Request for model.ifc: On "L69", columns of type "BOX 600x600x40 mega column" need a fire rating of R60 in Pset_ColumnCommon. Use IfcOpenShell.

First a look at what the model holds.

```python
import ifcopenshell
import ifcopenshell.util.element

model = ifcopenshell.open("model.ifc")
print(model.schema)
storey = next(s for s in model.by_type("IfcBuildingStorey") if s.Name == "L69")
columns = [e for e in ifcopenshell.util.element.get_decomposition(storey) if e.is_a("IfcColumn")]
seen = {}
for e in columns:
    element_type = ifcopenshell.util.element.get_type(e)
    key = (element_type.Name if element_type != e and element_type else None, ifcopenshell.util.element.get_pset(e, "Pset_ColumnCommon", "FireRating"))
    seen[key] = seen.get(key, 0) + 1
for (name, value), count in sorted(seen.items(), key=str):
    print(count, "x", name, "|", value)
```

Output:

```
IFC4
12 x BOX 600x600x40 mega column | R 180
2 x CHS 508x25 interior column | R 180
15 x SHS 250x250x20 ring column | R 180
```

```python
import ifcopenshell
import ifcopenshell.api.pset
import ifcopenshell.util.element

model = ifcopenshell.open("model.ifc")

storey = next(s for s in model.by_type("IfcBuildingStorey") if s.Name == "L69")
columns = [e for e in ifcopenshell.util.element.get_decomposition(storey) if e.is_a("IfcColumn")]

count = 0
for e in columns:
    element_type = ifcopenshell.util.element.get_type(e)
    if element_type in (None, e) or element_type.Name != "BOX 600x600x40 mega column":
        continue
    found = ifcopenshell.util.element.get_pset(e, "Pset_ColumnCommon", should_inherit=False)
    if found:
        pset = model.by_id(found["id"])
        if len(ifcopenshell.util.element.get_elements_by_pset(pset)) > 1:
            pset = ifcopenshell.api.pset.unshare_pset(model, products=[e], pset=pset)[0]
    else:
        pset = ifcopenshell.api.pset.add_pset(model, product=e, name="Pset_ColumnCommon")
    ifcopenshell.api.pset.edit_pset(model, pset=pset, properties={"FireRating": "R60"})
    count += 1

print(count, "columns updated")

model.write("model_rev.ifc")
```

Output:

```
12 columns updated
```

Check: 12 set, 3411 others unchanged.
